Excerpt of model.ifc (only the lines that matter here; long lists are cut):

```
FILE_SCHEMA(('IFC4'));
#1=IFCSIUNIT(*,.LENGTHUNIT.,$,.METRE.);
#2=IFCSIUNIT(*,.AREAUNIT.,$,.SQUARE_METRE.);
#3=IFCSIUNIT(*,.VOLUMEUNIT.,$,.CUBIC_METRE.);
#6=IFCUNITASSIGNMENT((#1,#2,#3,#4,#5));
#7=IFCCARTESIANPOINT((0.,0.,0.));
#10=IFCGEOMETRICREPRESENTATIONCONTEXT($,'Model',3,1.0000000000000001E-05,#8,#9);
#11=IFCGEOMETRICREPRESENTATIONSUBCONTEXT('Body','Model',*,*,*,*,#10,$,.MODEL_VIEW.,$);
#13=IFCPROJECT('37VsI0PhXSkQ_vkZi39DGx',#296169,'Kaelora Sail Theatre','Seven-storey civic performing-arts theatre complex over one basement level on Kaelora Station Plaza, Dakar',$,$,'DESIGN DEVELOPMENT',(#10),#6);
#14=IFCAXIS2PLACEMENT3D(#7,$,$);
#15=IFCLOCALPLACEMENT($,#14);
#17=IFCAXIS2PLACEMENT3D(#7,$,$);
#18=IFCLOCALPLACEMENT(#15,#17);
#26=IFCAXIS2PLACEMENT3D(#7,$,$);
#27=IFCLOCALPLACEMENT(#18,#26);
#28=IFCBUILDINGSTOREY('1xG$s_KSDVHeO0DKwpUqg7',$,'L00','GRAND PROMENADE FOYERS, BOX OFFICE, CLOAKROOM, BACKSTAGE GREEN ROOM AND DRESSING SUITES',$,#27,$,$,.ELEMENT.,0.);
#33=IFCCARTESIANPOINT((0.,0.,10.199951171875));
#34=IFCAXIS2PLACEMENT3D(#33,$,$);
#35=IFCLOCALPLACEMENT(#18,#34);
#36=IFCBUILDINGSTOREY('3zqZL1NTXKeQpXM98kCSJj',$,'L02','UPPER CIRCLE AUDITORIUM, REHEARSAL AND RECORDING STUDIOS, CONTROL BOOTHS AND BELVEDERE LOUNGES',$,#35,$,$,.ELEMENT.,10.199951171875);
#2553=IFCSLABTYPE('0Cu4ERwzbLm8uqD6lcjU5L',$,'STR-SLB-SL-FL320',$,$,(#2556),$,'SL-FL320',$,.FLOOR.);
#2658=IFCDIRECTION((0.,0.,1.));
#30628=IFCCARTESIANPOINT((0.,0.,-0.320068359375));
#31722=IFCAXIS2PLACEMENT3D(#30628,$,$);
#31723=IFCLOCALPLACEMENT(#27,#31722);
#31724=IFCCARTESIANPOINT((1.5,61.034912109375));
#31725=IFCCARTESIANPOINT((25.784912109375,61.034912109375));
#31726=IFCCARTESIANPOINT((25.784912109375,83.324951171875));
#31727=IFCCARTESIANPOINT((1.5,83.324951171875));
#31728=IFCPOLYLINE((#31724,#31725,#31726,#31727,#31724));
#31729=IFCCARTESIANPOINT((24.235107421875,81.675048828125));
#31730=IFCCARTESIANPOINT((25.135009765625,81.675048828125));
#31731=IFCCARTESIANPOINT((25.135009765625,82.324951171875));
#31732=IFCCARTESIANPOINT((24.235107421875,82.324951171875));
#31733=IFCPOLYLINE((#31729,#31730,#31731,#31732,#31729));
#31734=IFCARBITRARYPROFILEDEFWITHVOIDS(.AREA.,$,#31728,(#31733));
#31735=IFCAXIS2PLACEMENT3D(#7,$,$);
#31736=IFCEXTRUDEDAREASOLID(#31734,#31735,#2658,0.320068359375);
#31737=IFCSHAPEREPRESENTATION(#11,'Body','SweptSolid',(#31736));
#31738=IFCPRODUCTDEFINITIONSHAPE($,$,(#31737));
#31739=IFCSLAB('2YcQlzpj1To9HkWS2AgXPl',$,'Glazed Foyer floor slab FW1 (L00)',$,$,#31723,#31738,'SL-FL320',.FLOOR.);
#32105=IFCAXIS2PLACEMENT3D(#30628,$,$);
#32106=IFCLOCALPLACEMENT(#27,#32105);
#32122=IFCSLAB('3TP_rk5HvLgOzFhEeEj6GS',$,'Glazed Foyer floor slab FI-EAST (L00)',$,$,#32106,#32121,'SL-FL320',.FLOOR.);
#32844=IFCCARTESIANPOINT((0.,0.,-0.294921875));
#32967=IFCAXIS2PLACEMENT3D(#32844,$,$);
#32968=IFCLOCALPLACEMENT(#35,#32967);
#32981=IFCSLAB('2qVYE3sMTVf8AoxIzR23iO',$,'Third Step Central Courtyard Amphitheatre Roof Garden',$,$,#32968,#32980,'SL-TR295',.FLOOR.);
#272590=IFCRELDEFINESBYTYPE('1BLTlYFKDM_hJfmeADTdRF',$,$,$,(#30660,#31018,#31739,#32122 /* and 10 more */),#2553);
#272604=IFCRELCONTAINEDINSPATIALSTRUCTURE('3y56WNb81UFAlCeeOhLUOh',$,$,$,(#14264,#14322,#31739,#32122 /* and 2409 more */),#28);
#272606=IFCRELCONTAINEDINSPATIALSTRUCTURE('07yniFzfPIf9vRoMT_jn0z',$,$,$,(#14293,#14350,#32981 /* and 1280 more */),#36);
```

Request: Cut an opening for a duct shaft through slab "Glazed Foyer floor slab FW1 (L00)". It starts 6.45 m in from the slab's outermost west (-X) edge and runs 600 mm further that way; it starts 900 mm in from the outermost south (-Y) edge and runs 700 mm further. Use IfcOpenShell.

```python
import numpy as np
import ifcopenshell
import ifcopenshell.api.feature
import ifcopenshell.api.geometry
import ifcopenshell.api.root
import ifcopenshell.geom
import ifcopenshell.util.placement
import ifcopenshell.util.representation
import ifcopenshell.util.shape
import ifcopenshell.util.unit

model = ifcopenshell.open("model.ifc")
unit_scale = ifcopenshell.util.unit.calculate_unit_scale(model)
settings = ifcopenshell.geom.settings()


def volume(element):
    """Net volume in cubic metres, openings subtracted."""
    shape = ifcopenshell.geom.create_shape(settings, element)
    return ifcopenshell.util.shape.get_volume(shape.geometry)


slab = model.by_guid("2YcQlzpj1To9HkWS2AgXPl")
before = volume(slab)

# Extent in the slab's own axes, in metres. The edges named are its -X and -Y sides.
slab_shape = ifcopenshell.geom.create_shape(settings, slab)
vertices = ifcopenshell.util.shape.get_vertices(slab_shape.geometry)
x_min, y_min, bottom = vertices.min(axis=0)
top = vertices[:, 2].max()

opening = ifcopenshell.api.root.create_entity(model, ifc_class="IfcOpeningElement", name="Duct shaft opening", predefined_type="OPENING")
context = ifcopenshell.util.representation.get_context(model, "Model", "Body", "MODEL_VIEW")
width, depth = 0.6, 0.7
outline = [(0.0, 0.0), (width, 0.0), (width, depth), (0.0, depth), (0.0, 0.0)]
# Overshoot both faces by 50 mm so the cut is clean.
shape = ifcopenshell.api.geometry.add_slab_representation(
    model, context=context, depth=top - bottom + 0.1, polyline=outline
)
ifcopenshell.api.geometry.assign_representation(model, product=opening, representation=shape)

matrix = ifcopenshell.util.placement.get_local_placement(slab.ObjectPlacement)
matrix[:, 3] = matrix @ np.append(np.array([x_min + 6.45, y_min + 0.9, bottom - 0.05]) / unit_scale, 1.0)
ifcopenshell.api.geometry.edit_object_placement(model, product=opening, matrix=matrix, is_si=False)
ifcopenshell.api.feature.add_feature(model, feature=opening, element=slab)

after = volume(slab)

print(f"slab volume {before:.3f} -> {after:.3f} m3")

model.write("model-out.ifc")
```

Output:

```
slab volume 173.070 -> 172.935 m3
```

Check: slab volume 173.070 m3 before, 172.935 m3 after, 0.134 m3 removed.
